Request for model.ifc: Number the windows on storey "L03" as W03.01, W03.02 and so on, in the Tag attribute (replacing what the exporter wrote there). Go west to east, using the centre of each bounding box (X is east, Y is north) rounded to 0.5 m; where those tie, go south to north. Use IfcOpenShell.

First a look at what the model holds.

```python
import ifcopenshell
import ifcopenshell.util.element
import ifcopenshell.util.placement

model = ifcopenshell.open("model.ifc")
print(model.schema)
storey = next(s for s in model.by_type("IfcBuildingStorey") if s.Name == "L03")
windows = [e for e in ifcopenshell.util.element.get_decomposition(storey) if e.is_a("IfcWindow")]
for e in sorted(windows, key=lambda e: e.id()):
    origin = ifcopenshell.util.placement.get_local_placement(e.ObjectPlacement)[:3, 3]
    print(e.id(), e.Tag, e.Name, origin.round(2) + 0.0, sep=" | ")
```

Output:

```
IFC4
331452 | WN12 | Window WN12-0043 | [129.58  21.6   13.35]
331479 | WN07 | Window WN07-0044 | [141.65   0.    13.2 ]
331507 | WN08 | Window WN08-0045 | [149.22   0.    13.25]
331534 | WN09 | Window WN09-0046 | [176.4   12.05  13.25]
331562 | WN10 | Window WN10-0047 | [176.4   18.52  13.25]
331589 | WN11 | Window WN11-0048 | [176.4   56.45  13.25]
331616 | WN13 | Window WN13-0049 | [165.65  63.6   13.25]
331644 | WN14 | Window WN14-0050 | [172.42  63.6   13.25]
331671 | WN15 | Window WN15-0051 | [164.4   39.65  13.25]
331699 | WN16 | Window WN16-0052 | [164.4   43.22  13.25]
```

```python
import ifcopenshell
import ifcopenshell.geom
import ifcopenshell.util.element
import ifcopenshell.util.shape

model = ifcopenshell.open("model.ifc")
settings = ifcopenshell.geom.settings()
settings.set("use-world-coords", True)


def centre(element):
    shape = ifcopenshell.geom.create_shape(settings, element)
    return ifcopenshell.util.shape.get_bbox_centroid(shape.geometry)


storey = next(s for s in model.by_type("IfcBuildingStorey") if s.Name == "L03")
windows = [e for e in ifcopenshell.util.element.get_decomposition(storey) if e.is_a("IfcWindow")]

# Insertion points can sit at a corner or the storey origin, so sort by the geometry (in metres).
centres = {e: centre(e) for e in windows}
windows.sort(key=lambda e: (round(centres[e][0] / 0.5), centres[e][1]))

for i, e in enumerate(windows, start=1):
    number = f"W03.{i:02d}"
    e.Tag = number
    print(e.id(), number)

model.write("model_updated.ifc")
```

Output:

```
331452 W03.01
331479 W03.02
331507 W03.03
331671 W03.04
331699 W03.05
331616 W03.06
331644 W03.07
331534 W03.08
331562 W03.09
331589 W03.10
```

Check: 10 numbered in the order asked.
